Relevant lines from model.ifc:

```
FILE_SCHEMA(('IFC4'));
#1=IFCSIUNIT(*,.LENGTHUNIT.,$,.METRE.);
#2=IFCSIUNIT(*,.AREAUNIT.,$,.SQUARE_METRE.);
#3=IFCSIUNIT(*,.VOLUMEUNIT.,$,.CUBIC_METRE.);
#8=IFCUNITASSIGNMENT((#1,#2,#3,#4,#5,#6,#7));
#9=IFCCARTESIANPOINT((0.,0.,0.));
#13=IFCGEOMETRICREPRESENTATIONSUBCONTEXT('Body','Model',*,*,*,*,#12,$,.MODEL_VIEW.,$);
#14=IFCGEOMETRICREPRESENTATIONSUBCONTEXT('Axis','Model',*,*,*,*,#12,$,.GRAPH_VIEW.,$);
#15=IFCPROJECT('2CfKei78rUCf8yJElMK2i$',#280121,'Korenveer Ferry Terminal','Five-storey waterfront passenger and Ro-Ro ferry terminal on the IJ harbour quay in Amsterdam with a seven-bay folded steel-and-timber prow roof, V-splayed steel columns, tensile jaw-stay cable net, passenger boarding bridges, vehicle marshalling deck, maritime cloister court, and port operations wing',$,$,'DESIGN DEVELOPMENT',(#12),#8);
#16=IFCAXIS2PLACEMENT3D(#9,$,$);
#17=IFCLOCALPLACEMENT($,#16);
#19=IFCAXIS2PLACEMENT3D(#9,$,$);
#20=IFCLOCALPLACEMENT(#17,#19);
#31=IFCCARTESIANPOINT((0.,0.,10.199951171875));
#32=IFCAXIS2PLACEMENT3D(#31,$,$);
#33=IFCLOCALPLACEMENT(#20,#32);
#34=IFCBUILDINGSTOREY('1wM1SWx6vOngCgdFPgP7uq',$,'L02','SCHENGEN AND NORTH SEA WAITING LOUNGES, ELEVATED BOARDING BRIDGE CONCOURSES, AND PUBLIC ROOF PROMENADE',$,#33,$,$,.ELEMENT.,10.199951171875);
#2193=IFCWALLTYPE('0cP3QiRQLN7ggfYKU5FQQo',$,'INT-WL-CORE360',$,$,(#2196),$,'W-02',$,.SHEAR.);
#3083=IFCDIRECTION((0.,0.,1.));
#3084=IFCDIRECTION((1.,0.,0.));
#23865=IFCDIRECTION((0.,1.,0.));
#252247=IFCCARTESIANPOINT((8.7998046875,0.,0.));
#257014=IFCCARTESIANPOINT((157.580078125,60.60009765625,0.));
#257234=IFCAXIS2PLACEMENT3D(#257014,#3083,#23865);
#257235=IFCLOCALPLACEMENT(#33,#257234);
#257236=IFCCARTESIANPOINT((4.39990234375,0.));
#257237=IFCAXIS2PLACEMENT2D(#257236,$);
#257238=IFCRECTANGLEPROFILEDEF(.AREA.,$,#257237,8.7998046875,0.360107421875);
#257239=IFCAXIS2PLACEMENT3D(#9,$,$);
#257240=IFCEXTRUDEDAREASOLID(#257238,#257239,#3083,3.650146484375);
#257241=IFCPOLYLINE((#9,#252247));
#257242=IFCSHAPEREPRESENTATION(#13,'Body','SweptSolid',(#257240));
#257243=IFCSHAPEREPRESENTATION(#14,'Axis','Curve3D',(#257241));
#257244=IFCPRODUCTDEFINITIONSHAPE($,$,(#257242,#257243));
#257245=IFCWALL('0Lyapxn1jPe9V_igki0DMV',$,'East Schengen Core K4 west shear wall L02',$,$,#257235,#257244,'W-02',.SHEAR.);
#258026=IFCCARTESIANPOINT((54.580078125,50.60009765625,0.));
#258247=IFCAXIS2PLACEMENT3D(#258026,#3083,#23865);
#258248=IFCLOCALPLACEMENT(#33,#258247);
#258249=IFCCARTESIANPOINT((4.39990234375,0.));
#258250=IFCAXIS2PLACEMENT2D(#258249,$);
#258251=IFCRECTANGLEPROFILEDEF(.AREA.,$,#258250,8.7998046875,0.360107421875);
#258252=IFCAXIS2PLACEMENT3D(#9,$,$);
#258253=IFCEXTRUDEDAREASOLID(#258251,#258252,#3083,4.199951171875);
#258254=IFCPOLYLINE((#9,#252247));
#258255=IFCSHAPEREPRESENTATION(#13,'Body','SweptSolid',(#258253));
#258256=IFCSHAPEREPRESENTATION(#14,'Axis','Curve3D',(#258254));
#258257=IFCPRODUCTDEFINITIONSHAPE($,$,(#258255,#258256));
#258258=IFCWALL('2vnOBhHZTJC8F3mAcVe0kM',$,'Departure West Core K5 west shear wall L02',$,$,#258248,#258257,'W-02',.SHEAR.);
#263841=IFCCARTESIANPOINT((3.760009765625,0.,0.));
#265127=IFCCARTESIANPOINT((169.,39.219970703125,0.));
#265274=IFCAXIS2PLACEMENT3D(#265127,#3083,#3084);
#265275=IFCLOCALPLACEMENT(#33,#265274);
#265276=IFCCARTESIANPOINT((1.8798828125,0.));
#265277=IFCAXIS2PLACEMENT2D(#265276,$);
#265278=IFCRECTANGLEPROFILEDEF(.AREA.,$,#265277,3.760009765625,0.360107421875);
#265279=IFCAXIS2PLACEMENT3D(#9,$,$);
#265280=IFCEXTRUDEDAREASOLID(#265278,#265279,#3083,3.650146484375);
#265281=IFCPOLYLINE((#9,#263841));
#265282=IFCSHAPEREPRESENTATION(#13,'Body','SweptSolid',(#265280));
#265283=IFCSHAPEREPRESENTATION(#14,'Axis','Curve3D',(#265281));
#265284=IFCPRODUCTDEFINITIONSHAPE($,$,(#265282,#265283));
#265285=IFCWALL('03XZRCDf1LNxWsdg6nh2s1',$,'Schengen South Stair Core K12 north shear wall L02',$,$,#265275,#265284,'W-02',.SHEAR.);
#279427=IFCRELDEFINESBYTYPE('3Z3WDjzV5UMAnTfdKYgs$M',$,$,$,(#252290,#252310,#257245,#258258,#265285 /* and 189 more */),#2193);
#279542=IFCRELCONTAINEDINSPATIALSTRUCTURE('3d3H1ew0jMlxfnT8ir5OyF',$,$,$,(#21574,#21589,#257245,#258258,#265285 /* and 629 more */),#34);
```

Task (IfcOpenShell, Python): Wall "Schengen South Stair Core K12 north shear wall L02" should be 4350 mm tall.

```python
import ifcopenshell
import ifcopenshell.geom
import ifcopenshell.util.representation
import ifcopenshell.util.shape
import ifcopenshell.util.unit

model = ifcopenshell.open("model.ifc")
unit_scale = ifcopenshell.util.unit.calculate_unit_scale(model)
settings = ifcopenshell.geom.settings()


def volume(element):
    """Net volume in cubic metres, openings subtracted."""
    shape = ifcopenshell.geom.create_shape(settings, element)
    return ifcopenshell.util.shape.get_volume(shape.geometry)


wall = model.by_guid("03XZRCDf1LNxWsdg6nh2s1")
before = volume(wall)

body = ifcopenshell.util.representation.get_representation(wall, "Model", "Body")
solid = body.Items[0]
old_height = solid.Depth
solid.Depth = 4.35 / unit_scale
after = volume(wall)

print(f"height {old_height:g} -> {solid.Depth:g}, volume {before:.3f} -> {after:.3f} m3")

model.write("model_rev.ifc")
```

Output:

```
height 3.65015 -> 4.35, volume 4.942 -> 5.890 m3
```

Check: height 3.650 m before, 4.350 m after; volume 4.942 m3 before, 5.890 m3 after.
